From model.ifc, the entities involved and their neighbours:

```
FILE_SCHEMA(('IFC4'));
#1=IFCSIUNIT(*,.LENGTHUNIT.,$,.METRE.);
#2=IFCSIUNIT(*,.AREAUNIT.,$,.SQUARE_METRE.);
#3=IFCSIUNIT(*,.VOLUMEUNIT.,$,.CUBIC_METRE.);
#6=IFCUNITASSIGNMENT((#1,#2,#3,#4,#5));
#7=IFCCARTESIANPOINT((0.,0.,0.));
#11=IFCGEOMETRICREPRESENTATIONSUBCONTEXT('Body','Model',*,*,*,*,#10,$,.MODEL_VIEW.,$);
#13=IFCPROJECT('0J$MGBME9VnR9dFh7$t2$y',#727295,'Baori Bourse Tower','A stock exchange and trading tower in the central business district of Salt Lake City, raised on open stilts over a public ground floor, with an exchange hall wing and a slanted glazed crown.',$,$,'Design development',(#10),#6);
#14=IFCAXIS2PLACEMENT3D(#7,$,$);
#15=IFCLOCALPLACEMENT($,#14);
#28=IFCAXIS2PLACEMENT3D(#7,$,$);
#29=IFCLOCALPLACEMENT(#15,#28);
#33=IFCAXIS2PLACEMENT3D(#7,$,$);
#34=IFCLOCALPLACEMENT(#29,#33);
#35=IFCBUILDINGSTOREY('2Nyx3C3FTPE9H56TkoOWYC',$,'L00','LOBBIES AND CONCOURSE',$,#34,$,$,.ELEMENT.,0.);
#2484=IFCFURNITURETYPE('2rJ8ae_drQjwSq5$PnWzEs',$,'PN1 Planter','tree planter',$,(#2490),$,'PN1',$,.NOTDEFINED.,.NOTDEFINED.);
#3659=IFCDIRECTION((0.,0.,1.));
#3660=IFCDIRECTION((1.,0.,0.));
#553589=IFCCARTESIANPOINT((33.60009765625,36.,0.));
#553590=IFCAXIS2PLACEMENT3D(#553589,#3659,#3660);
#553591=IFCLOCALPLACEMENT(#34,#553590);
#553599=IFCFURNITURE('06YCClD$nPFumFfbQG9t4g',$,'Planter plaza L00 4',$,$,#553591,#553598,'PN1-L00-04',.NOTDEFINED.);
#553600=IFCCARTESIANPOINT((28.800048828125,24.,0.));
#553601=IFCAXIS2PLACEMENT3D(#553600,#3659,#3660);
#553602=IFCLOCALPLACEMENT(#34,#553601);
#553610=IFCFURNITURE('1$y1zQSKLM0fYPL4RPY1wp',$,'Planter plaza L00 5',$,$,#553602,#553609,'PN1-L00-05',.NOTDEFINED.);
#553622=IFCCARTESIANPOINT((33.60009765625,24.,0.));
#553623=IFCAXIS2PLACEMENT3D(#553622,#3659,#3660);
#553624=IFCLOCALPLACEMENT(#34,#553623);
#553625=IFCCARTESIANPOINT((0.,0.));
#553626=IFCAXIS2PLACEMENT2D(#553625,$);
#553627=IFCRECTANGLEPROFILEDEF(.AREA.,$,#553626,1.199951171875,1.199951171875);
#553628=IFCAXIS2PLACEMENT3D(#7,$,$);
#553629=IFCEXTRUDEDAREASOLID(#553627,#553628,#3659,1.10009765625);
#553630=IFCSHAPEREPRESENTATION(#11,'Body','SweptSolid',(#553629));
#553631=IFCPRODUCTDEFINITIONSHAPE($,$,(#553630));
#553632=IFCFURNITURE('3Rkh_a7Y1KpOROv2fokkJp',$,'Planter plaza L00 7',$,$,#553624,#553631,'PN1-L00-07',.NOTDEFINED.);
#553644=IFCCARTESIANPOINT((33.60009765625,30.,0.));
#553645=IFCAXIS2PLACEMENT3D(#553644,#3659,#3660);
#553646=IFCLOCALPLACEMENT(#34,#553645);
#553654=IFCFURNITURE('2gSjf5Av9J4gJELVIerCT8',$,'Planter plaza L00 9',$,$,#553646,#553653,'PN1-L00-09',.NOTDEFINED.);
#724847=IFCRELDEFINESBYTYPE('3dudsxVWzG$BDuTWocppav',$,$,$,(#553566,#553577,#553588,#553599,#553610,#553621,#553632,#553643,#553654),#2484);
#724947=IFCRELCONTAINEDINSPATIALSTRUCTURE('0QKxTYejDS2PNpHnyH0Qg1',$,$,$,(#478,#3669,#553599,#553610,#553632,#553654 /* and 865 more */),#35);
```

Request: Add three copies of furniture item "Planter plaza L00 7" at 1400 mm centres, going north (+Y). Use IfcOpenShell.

```python
import numpy as np
import ifcopenshell
import ifcopenshell.api.geometry
import ifcopenshell.api.root
import ifcopenshell.util.element
import ifcopenshell.util.placement
import ifcopenshell.util.unit

model = ifcopenshell.open("model.ifc")
unit_scale = ifcopenshell.util.unit.calculate_unit_scale(model)

source = model.by_guid("3Rkh_a7Y1KpOROv2fokkJp")
base = ifcopenshell.util.placement.get_local_placement(source.ObjectPlacement)
step = np.array([0.0, 1.0, 0.0]) * 1.4 / unit_scale

for i in range(1, 4):
    copy = ifcopenshell.api.root.copy_class(model, product=source)
    copy.Representation = ifcopenshell.util.element.copy_deep(
        model, source.Representation, exclude=["IfcGeometricRepresentationContext", "IfcRepresentationMap"]
    )
    copy.Tag = None
    matrix = base.copy()
    matrix[:3, 3] += i * step
    print("added at", matrix[:3, 3].round(3) + 0.0)
    ifcopenshell.api.geometry.edit_object_placement(model, product=copy, matrix=matrix, is_si=False)

model.write("model_rev.ifc")
```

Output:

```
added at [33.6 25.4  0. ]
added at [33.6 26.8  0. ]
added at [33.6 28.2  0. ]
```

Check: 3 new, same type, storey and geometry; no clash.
